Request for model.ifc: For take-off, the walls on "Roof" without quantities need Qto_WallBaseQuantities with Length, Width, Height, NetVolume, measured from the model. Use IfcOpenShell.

First a look at what the model holds.

```python
import ifcopenshell
import ifcopenshell.util.element
import ifcopenshell.util.unit

model = ifcopenshell.open("model.ifc")
print(model.schema)
for unit_type in ("LENGTHUNIT", "AREAUNIT", "VOLUMEUNIT"):
    print(unit_type, ifcopenshell.util.unit.calculate_unit_scale(model, unit_type))
storey = next(s for s in model.by_type("IfcBuildingStorey") if s.Name == "Roof")
walls = [e for e in ifcopenshell.util.element.get_decomposition(storey) if e.is_a("IfcWall")]
for e in sorted(walls, key=lambda e: e.id()):
    print(e.id(), e.is_a(), e.Name, list(ifcopenshell.util.element.get_psets(e, qtos_only=True)), sep=" | ")
```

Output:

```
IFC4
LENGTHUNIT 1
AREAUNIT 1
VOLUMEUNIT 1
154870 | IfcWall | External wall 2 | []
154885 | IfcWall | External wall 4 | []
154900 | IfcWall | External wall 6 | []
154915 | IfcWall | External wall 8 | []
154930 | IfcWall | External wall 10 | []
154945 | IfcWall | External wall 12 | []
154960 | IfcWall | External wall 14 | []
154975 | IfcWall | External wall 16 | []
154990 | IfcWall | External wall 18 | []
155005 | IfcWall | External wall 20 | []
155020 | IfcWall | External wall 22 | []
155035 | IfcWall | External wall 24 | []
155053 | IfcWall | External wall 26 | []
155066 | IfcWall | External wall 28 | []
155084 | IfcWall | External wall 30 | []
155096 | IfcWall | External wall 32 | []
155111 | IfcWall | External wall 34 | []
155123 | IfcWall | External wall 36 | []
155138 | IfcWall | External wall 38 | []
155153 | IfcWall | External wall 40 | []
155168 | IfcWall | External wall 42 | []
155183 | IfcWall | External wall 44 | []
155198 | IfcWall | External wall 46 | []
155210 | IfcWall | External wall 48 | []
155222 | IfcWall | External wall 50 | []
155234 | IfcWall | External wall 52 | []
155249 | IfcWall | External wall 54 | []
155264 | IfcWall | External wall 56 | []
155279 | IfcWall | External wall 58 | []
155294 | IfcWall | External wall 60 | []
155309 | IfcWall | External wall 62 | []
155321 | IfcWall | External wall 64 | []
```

```python
import ifcopenshell
import ifcopenshell.api.pset
import ifcopenshell.geom
import ifcopenshell.util.element
import ifcopenshell.util.shape
import ifcopenshell.util.unit

model = ifcopenshell.open("model.ifc")
unit_scale = ifcopenshell.util.unit.calculate_unit_scale(model)
volume_scale = ifcopenshell.util.unit.calculate_unit_scale(model, "VOLUMEUNIT")
settings = ifcopenshell.geom.settings()

storey = next(s for s in model.by_type("IfcBuildingStorey") if s.Name == "Roof")
walls = [e for e in ifcopenshell.util.element.get_decomposition(storey) if e.is_a("IfcWall")]

for e in sorted(walls, key=lambda e: e.id()):
    if ifcopenshell.util.element.get_psets(e, qtos_only=True, should_inherit=False):
        continue
    # Geometry comes back in metres, in the element's own axes.
    shape = ifcopenshell.geom.create_shape(settings, e)
    values = {
        "Length": ifcopenshell.util.shape.get_x(shape.geometry) / unit_scale,
        "Width": ifcopenshell.util.shape.get_y(shape.geometry) / unit_scale,
        "Height": ifcopenshell.util.shape.get_z(shape.geometry) / unit_scale,
        "NetVolume": ifcopenshell.util.shape.get_volume(shape.geometry) / volume_scale,
    }
    qto = ifcopenshell.api.pset.add_qto(model, product=e, name="Qto_WallBaseQuantities")
    ifcopenshell.api.pset.edit_qto(model, qto=qto, properties=values)
    print(e.id(), {k: round(v, 3) for k, v in values.items()})

model.write("model_v2.ifc")
```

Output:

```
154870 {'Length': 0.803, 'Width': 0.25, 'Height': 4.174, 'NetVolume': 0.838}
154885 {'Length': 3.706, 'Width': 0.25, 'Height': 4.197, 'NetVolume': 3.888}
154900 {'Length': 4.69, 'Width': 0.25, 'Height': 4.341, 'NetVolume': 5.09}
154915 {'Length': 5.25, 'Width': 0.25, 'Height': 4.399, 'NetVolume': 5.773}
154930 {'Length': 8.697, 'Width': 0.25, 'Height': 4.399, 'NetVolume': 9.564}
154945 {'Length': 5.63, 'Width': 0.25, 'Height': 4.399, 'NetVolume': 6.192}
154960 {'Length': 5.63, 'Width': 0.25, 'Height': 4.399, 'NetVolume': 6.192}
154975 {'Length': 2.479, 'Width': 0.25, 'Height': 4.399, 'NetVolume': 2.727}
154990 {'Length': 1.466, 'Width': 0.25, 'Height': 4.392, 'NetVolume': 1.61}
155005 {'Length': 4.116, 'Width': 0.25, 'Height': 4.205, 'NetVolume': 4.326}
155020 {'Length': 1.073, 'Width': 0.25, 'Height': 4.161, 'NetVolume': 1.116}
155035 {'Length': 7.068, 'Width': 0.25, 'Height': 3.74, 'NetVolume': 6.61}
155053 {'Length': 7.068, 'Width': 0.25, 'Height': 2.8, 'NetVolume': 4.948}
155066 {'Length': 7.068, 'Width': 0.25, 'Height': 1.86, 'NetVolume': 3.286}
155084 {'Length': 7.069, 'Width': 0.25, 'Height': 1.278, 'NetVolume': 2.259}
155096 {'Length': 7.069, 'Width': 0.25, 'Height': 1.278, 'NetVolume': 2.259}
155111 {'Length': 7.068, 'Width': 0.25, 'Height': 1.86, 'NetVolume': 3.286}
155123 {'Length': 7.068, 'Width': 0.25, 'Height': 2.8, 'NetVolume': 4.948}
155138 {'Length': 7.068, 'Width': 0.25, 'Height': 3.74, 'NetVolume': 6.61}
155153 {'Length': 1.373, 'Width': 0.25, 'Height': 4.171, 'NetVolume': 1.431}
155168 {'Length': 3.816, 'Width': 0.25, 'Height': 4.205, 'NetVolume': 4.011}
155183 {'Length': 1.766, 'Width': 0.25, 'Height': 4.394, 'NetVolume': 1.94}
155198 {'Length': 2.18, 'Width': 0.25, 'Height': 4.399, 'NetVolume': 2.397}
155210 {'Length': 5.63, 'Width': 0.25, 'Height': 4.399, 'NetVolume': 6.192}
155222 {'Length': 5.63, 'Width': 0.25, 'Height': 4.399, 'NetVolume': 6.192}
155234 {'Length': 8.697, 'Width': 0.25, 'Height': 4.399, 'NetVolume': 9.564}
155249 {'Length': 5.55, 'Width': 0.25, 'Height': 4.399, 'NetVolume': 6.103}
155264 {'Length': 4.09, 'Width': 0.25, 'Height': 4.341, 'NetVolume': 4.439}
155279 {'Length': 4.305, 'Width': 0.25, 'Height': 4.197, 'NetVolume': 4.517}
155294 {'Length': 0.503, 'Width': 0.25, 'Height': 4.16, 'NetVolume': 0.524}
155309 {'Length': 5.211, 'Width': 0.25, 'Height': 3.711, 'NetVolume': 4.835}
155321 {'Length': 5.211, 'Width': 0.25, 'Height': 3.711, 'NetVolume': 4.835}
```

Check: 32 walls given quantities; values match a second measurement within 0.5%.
